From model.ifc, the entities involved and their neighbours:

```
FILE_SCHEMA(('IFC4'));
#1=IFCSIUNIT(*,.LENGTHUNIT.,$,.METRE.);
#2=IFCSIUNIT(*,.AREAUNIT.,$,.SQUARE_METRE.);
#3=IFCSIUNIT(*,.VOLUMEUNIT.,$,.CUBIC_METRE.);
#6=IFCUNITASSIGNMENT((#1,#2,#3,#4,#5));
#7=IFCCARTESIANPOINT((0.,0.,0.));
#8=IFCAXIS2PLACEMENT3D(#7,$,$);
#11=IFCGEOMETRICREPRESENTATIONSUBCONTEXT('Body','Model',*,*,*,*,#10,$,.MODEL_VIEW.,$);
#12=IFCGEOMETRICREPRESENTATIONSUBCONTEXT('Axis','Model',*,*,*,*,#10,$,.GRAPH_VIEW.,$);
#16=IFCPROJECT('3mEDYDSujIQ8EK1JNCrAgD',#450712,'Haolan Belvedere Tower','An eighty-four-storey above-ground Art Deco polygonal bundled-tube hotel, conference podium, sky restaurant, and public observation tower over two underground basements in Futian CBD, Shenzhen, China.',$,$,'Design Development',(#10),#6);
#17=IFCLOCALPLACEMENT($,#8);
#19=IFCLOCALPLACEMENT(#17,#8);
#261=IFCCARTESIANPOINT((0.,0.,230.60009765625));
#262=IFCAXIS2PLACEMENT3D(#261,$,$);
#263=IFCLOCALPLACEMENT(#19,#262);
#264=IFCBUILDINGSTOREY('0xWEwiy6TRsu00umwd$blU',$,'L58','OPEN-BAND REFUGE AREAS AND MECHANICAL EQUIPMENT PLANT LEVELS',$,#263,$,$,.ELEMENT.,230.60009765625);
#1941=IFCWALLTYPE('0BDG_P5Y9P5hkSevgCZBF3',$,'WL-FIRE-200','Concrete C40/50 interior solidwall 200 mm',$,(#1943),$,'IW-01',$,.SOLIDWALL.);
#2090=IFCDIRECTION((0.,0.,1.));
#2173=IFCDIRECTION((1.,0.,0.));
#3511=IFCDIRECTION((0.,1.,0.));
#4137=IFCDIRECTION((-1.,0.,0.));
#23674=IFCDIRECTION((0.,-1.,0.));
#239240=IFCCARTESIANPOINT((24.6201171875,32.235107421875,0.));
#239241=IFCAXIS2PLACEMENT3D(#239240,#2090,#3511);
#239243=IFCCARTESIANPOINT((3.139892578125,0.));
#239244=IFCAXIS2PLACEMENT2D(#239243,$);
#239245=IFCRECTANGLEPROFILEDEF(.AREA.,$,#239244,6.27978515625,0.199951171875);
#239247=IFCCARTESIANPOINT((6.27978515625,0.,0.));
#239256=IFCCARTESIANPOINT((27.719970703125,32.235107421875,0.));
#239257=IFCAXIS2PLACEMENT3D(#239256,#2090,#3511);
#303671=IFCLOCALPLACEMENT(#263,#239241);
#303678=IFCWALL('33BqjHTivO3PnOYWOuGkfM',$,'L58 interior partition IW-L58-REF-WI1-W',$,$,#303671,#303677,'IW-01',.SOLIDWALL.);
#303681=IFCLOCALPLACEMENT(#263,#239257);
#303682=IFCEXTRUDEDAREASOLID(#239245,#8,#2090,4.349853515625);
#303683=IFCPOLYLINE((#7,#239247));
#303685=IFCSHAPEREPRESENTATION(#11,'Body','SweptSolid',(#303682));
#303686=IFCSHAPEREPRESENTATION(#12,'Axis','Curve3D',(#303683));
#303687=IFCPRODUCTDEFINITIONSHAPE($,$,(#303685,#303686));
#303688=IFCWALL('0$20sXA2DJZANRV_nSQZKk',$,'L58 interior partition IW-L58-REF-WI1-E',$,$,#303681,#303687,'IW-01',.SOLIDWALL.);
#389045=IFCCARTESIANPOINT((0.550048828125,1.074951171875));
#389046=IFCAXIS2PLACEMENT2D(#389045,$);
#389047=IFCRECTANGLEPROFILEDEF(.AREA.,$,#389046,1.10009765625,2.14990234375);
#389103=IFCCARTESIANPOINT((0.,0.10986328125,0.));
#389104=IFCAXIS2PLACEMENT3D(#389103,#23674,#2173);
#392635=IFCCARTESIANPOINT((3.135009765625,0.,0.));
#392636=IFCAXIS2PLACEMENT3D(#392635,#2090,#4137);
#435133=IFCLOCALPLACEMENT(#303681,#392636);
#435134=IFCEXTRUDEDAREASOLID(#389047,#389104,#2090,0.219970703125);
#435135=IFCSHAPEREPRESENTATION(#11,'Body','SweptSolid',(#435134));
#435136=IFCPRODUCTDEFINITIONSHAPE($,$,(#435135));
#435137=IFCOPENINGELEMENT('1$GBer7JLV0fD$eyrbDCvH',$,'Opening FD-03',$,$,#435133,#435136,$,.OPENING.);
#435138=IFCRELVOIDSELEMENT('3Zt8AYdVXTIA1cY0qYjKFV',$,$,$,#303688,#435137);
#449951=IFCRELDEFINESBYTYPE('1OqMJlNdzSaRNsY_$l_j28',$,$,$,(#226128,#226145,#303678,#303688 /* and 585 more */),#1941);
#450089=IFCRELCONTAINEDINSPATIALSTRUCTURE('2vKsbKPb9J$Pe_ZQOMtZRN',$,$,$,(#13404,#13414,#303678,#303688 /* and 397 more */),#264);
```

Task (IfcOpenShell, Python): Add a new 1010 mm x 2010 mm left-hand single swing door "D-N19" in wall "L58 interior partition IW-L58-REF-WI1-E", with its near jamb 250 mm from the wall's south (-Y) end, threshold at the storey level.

```python
import numpy as np
import ifcopenshell
import ifcopenshell.api.feature
import ifcopenshell.api.geometry
import ifcopenshell.api.root
import ifcopenshell.api.spatial
import ifcopenshell.geom
import ifcopenshell.util.element
import ifcopenshell.util.placement
import ifcopenshell.util.representation
import ifcopenshell.util.shape
import ifcopenshell.util.unit

model = ifcopenshell.open("model.ifc")
unit_scale = ifcopenshell.util.unit.calculate_unit_scale(model)
settings = ifcopenshell.geom.settings()


def volume(element):
    """Net volume in cubic metres, openings subtracted."""
    shape = ifcopenshell.geom.create_shape(settings, element)
    return ifcopenshell.util.shape.get_volume(shape.geometry)


wall = model.by_guid("0$20sXA2DJZANRV_nSQZKk")
storey = ifcopenshell.util.element.get_container(wall, ifc_class="IfcBuildingStorey")
context = ifcopenshell.util.representation.get_context(model, "Model", "Body", "MODEL_VIEW")
before = volume(wall)

width, height, from_end, sill = 1.01, 2.01, 0.25, 0.0  # metres

# The wall runs along its own X axis, and the end named is its -X end.
wall_shape = ifcopenshell.geom.create_shape(settings, wall)
x, y, z = ifcopenshell.util.shape.get_vertices(wall_shape.geometry).T
start = x.min() + from_end
face, thickness = float(y.min()), float(y.max() - y.min())
wall_matrix = ifcopenshell.util.placement.get_local_placement(wall.ObjectPlacement)
level = ifcopenshell.util.placement.get_local_placement(storey.ObjectPlacement)[2, 3]


def in_wall(x, y):
    """Placement at x, y metres in the wall's axes, at sill height."""
    matrix = wall_matrix.copy()
    matrix[:, 3] = wall_matrix @ np.array([x / unit_scale, y / unit_scale, 0.0, 1.0])
    matrix[2, 3] = level + sill / unit_scale
    return matrix


# Opening: a box that overshoots both wall faces by 50 mm.
opening = ifcopenshell.api.root.create_entity(model, ifc_class="IfcOpeningElement", predefined_type="OPENING")
box = ifcopenshell.api.geometry.add_wall_representation(
    model, context=context, length=width, height=height, thickness=thickness + 0.1
)
ifcopenshell.api.geometry.assign_representation(model, product=opening, representation=box)
ifcopenshell.api.geometry.edit_object_placement(model, product=opening, matrix=in_wall(start, face - 0.05), is_si=False)
ifcopenshell.api.feature.add_feature(model, feature=opening, element=wall)

door = ifcopenshell.api.root.create_entity(model, ifc_class="IfcDoor", name="D-N19", predefined_type="DOOR")
door.OverallWidth, door.OverallHeight = width / unit_scale, height / unit_scale
door.OperationType = "SINGLE_SWING_LEFT"
body = ifcopenshell.api.geometry.add_door_representation(
    model,
    context=context,
    overall_width=door.OverallWidth,
    overall_height=door.OverallHeight,
    operation_type="SINGLE_SWING_LEFT",
    lining_properties={"LiningDepth": thickness / unit_scale, "ThresholdDepth": thickness / unit_scale},
)
ifcopenshell.api.geometry.assign_representation(model, product=door, representation=body)
ifcopenshell.api.spatial.assign_container(model, products=[door], relating_structure=storey)
ifcopenshell.api.feature.add_filling(model, opening=opening, element=door)

# The lining spans the wall, so the door starts at the wall face.
ifcopenshell.api.geometry.edit_object_placement(model, product=door, matrix=in_wall(start, face), is_si=False)

after = volume(wall)

print(f"wall volume {before:.3f} -> {after:.3f} m3")

model.write("model_edited.ifc")
```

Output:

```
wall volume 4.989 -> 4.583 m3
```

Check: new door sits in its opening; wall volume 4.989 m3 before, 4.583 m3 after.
